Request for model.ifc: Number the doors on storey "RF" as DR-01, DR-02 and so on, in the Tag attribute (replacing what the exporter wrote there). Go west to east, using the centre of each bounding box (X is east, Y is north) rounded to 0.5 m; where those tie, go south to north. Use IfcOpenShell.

First a look at what the model holds.

```python
import ifcopenshell
import ifcopenshell.util.element
import ifcopenshell.util.placement

model = ifcopenshell.open("model.ifc")
print(model.schema)
storey = next(s for s in model.by_type("IfcBuildingStorey") if s.Name == "RF")
doors = [e for e in ifcopenshell.util.element.get_decomposition(storey) if e.is_a("IfcDoor")]
for e in sorted(doors, key=lambda e: e.id()):
    origin = ifcopenshell.util.placement.get_local_placement(e.ObjectPlacement)[:3, 3]
    print(e.id(), e.Tag, e.Name, origin.round(2) + 0.0, sep=" | ")
```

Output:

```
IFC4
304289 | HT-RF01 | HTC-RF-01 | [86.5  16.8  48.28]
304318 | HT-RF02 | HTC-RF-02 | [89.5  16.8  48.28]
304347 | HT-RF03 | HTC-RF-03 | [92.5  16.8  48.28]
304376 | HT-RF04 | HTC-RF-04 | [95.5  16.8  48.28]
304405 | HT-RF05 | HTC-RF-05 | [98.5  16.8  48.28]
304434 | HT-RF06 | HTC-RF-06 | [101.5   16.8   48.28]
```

```python
import ifcopenshell
import ifcopenshell.geom
import ifcopenshell.util.element
import ifcopenshell.util.shape

model = ifcopenshell.open("model.ifc")
settings = ifcopenshell.geom.settings()
settings.set("use-world-coords", True)


def centre(element):
    shape = ifcopenshell.geom.create_shape(settings, element)
    return ifcopenshell.util.shape.get_bbox_centroid(shape.geometry)


storey = next(s for s in model.by_type("IfcBuildingStorey") if s.Name == "RF")
doors = [e for e in ifcopenshell.util.element.get_decomposition(storey) if e.is_a("IfcDoor")]

# Insertion points can sit at a corner or the storey origin, so sort by the geometry (in metres).
centres = {e: centre(e) for e in doors}
doors.sort(key=lambda e: (round(centres[e][0] / 0.5), centres[e][1]))

for i, e in enumerate(doors, start=1):
    number = f"DR-{i:02d}"
    e.Tag = number
    print(e.id(), number)

model.write("model-out.ifc")
```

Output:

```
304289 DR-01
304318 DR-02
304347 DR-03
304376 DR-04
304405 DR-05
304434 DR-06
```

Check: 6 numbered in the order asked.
